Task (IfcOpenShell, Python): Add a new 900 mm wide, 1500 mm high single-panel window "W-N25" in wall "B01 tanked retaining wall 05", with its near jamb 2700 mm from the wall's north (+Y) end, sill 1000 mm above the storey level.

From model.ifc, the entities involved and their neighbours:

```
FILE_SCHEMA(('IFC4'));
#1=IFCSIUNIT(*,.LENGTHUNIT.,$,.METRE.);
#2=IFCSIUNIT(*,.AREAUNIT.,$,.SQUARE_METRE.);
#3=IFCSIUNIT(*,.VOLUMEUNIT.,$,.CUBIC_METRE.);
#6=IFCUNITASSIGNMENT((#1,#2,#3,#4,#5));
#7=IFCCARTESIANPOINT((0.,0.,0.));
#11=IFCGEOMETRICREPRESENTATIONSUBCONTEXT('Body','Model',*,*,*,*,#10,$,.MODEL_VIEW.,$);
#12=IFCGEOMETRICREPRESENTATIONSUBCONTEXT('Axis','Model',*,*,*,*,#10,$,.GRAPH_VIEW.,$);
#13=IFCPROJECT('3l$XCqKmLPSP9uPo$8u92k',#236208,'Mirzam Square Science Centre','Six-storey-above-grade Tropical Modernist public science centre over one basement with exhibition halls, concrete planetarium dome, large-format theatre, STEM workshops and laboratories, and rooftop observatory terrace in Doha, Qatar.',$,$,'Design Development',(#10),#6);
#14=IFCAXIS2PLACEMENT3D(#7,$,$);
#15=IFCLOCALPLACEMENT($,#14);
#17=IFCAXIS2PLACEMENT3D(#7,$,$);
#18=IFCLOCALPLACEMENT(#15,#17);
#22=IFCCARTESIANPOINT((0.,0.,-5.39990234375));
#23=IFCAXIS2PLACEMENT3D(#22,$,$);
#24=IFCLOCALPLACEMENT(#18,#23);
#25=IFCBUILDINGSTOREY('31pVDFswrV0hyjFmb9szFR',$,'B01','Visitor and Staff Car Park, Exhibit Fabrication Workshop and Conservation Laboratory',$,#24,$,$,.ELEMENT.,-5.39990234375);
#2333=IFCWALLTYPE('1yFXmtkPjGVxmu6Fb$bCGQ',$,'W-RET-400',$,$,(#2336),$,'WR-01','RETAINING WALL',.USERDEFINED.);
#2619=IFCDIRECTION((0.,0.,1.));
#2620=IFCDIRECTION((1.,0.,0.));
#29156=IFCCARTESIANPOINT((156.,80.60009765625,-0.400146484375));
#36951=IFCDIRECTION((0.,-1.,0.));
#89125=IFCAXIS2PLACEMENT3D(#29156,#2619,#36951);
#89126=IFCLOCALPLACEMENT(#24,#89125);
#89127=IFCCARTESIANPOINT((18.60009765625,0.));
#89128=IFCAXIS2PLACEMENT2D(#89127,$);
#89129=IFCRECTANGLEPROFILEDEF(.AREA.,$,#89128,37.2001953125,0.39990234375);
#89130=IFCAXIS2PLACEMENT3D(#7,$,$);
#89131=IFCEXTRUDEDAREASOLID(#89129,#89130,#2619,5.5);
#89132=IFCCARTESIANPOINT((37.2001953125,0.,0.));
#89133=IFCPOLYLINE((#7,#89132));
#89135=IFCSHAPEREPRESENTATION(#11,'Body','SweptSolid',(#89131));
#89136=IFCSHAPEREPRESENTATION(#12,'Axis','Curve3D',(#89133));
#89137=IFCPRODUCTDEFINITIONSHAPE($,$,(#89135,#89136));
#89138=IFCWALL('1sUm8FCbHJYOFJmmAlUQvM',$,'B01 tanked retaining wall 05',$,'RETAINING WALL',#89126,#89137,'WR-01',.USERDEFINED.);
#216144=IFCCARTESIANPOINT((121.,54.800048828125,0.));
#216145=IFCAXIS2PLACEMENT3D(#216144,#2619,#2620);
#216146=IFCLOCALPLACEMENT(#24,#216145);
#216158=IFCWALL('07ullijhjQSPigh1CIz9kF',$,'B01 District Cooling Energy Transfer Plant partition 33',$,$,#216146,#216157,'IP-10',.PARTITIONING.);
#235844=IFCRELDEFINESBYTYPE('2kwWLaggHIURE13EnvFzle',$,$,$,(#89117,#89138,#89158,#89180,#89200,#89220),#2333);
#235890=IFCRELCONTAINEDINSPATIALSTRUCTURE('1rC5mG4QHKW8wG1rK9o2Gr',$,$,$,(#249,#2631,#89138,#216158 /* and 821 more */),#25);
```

```python
import numpy as np
import ifcopenshell
import ifcopenshell.api.feature
import ifcopenshell.api.geometry
import ifcopenshell.api.root
import ifcopenshell.api.spatial
import ifcopenshell.geom
import ifcopenshell.util.element
import ifcopenshell.util.placement
import ifcopenshell.util.representation
import ifcopenshell.util.shape
import ifcopenshell.util.unit

model = ifcopenshell.open("model.ifc")
unit_scale = ifcopenshell.util.unit.calculate_unit_scale(model)
settings = ifcopenshell.geom.settings()


def volume(element):
    """Net volume in cubic metres, openings subtracted."""
    shape = ifcopenshell.geom.create_shape(settings, element)
    return ifcopenshell.util.shape.get_volume(shape.geometry)


wall = model.by_guid("1sUm8FCbHJYOFJmmAlUQvM")
storey = ifcopenshell.util.element.get_container(wall, ifc_class="IfcBuildingStorey")
context = ifcopenshell.util.representation.get_context(model, "Model", "Body", "MODEL_VIEW")
before = volume(wall)

width, height, from_end, sill = 0.9, 1.5, 2.7, 1  # metres

# The wall runs along its own X axis, and the end named is its -X end.
wall_shape = ifcopenshell.geom.create_shape(settings, wall)
x, y, z = ifcopenshell.util.shape.get_vertices(wall_shape.geometry).T
start = x.min() + from_end
face, thickness = float(y.min()), float(y.max() - y.min())
wall_matrix = ifcopenshell.util.placement.get_local_placement(wall.ObjectPlacement)
level = ifcopenshell.util.placement.get_local_placement(storey.ObjectPlacement)[2, 3]


def in_wall(x, y):
    """Placement at x, y metres in the wall's axes, at sill height."""
    matrix = wall_matrix.copy()
    matrix[:, 3] = wall_matrix @ np.array([x / unit_scale, y / unit_scale, 0.0, 1.0])
    matrix[2, 3] = level + sill / unit_scale
    return matrix


# Opening: a box that overshoots both wall faces by 50 mm.
opening = ifcopenshell.api.root.create_entity(model, ifc_class="IfcOpeningElement", predefined_type="OPENING")
box = ifcopenshell.api.geometry.add_wall_representation(
    model, context=context, length=width, height=height, thickness=thickness + 0.1
)
ifcopenshell.api.geometry.assign_representation(model, product=opening, representation=box)
ifcopenshell.api.geometry.edit_object_placement(model, product=opening, matrix=in_wall(start, face - 0.05), is_si=False)
ifcopenshell.api.feature.add_feature(model, feature=opening, element=wall)

window = ifcopenshell.api.root.create_entity(model, ifc_class="IfcWindow", name="W-N25", predefined_type="WINDOW")
window.OverallWidth, window.OverallHeight = width / unit_scale, height / unit_scale
window.PartitioningType = "SINGLE_PANEL"
body = ifcopenshell.api.geometry.add_window_representation(
    model,
    context=context,
    overall_width=window.OverallWidth,
    overall_height=window.OverallHeight,
    partition_type="SINGLE_PANEL",
)
ifcopenshell.api.geometry.assign_representation(model, product=window, representation=body)
ifcopenshell.api.spatial.assign_container(model, products=[window], relating_structure=storey)
ifcopenshell.api.feature.add_filling(model, opening=opening, element=window)

# Centre the window in the wall's thickness.
ifcopenshell.api.geometry.edit_object_placement(model, product=window, matrix=in_wall(start, face), is_si=False)
window_shape = ifcopenshell.geom.create_shape(settings, window)
depth = ifcopenshell.util.shape.get_vertices(window_shape.geometry)[:, 1]
offset = face + thickness / 2 - (depth.min() + depth.max()) / 2
ifcopenshell.api.geometry.edit_object_placement(model, product=window, matrix=in_wall(start, offset), is_si=False)

after = volume(wall)

print(f"wall volume {before:.3f} -> {after:.3f} m3")

model.write("model_rev.ifc")
```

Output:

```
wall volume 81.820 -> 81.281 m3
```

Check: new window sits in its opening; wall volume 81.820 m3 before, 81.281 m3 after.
